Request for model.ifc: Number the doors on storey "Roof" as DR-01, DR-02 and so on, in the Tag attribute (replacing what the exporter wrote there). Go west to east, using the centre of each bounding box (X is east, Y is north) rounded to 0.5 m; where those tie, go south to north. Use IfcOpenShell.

First a look at what the model holds.

```python
import ifcopenshell
import ifcopenshell.util.element
import ifcopenshell.util.placement

model = ifcopenshell.open("model.ifc")
print(model.schema)
storey = next(s for s in model.by_type("IfcBuildingStorey") if s.Name == "Roof")
doors = [e for e in ifcopenshell.util.element.get_decomposition(storey) if e.is_a("IfcDoor")]
for e in sorted(doors, key=lambda e: e.id()):
    origin = ifcopenshell.util.placement.get_local_placement(e.ObjectPlacement)[:3, 3]
    print(e.id(), e.Tag, e.Name, origin.round(2) + 0.0, sep=" | ")
```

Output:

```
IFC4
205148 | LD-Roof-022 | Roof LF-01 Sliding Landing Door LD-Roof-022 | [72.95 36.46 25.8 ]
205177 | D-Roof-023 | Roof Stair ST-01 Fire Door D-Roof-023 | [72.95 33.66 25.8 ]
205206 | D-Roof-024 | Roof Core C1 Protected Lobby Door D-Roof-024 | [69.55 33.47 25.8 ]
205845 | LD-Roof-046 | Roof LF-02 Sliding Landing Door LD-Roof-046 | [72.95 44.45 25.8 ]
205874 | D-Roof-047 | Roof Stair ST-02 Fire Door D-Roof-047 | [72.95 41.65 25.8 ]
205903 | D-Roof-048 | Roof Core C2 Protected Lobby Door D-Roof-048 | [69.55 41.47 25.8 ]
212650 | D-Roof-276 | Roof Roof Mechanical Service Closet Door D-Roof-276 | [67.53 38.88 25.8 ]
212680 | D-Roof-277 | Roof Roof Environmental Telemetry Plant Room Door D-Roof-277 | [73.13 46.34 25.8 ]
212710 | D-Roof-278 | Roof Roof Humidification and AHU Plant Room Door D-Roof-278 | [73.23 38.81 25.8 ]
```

```python
import ifcopenshell
import ifcopenshell.geom
import ifcopenshell.util.element
import ifcopenshell.util.shape

model = ifcopenshell.open("model.ifc")
settings = ifcopenshell.geom.settings()
settings.set("use-world-coords", True)


def centre(element):
    shape = ifcopenshell.geom.create_shape(settings, element)
    return ifcopenshell.util.shape.get_bbox_centroid(shape.geometry)


storey = next(s for s in model.by_type("IfcBuildingStorey") if s.Name == "Roof")
doors = [e for e in ifcopenshell.util.element.get_decomposition(storey) if e.is_a("IfcDoor")]

# Insertion points can sit at a corner or the storey origin, so sort by the geometry (in metres).
centres = {e: centre(e) for e in doors}
doors.sort(key=lambda e: (round(centres[e][0] / 0.5), centres[e][1]))

for i, e in enumerate(doors, start=1):
    number = f"DR-{i:02d}"
    e.Tag = number
    print(e.id(), number)

model.write("model_updated.ifc")
```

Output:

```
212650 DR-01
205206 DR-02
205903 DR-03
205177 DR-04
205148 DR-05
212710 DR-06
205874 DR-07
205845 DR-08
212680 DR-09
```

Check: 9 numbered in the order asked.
